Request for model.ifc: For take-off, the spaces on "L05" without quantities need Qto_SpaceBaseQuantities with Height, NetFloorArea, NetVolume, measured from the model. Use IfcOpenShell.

First a look at what the model holds.

```python
import ifcopenshell
import ifcopenshell.util.element
import ifcopenshell.util.unit

model = ifcopenshell.open("model.ifc")
print(model.schema)
for unit_type in ("LENGTHUNIT", "AREAUNIT", "VOLUMEUNIT"):
    print(unit_type, ifcopenshell.util.unit.calculate_unit_scale(model, unit_type))
storey = next(s for s in model.by_type("IfcBuildingStorey") if s.Name == "L05")
spaces = [e for e in ifcopenshell.util.element.get_decomposition(storey) if e.is_a("IfcSpace")]
for e in sorted(spaces, key=lambda e: e.id()):
    print(e.id(), e.is_a(), e.Name, list(ifcopenshell.util.element.get_psets(e, qtos_only=True)), sep=" | ")
```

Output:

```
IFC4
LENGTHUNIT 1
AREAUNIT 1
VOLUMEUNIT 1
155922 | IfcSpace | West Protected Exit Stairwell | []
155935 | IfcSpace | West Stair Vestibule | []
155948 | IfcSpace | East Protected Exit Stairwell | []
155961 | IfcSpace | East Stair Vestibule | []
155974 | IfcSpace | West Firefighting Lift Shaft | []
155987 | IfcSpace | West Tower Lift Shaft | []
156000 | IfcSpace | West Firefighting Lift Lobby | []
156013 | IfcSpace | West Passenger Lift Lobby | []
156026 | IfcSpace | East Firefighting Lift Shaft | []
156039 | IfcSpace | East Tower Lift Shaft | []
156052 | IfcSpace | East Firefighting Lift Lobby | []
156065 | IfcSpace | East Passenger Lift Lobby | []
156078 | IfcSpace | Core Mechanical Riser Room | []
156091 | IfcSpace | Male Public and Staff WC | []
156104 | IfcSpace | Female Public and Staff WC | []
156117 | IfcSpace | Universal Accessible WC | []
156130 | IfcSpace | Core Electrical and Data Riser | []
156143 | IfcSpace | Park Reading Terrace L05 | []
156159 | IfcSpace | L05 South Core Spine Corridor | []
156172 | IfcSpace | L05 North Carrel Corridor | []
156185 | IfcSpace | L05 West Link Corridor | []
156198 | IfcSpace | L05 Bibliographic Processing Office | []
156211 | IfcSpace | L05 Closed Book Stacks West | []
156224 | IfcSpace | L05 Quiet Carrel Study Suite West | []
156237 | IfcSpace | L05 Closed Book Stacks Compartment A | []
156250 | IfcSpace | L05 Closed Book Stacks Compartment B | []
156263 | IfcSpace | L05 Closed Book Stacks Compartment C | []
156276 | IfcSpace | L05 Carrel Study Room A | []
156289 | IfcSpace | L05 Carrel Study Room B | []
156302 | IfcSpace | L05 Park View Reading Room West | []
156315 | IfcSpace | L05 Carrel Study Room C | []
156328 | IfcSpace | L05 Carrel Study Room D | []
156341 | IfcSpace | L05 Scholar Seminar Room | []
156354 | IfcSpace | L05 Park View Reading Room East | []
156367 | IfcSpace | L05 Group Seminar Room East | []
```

```python
import ifcopenshell
import ifcopenshell.api.pset
import ifcopenshell.geom
import ifcopenshell.util.element
import ifcopenshell.util.shape
import ifcopenshell.util.unit

model = ifcopenshell.open("model.ifc")
unit_scale = ifcopenshell.util.unit.calculate_unit_scale(model)
area_scale = ifcopenshell.util.unit.calculate_unit_scale(model, "AREAUNIT")
volume_scale = ifcopenshell.util.unit.calculate_unit_scale(model, "VOLUMEUNIT")
settings = ifcopenshell.geom.settings()

storey = next(s for s in model.by_type("IfcBuildingStorey") if s.Name == "L05")
spaces = [e for e in ifcopenshell.util.element.get_decomposition(storey) if e.is_a("IfcSpace")]

for e in sorted(spaces, key=lambda e: e.id()):
    if ifcopenshell.util.element.get_psets(e, qtos_only=True, should_inherit=False):
        continue
    # Geometry comes back in metres, in the element's own axes.
    shape = ifcopenshell.geom.create_shape(settings, e)
    values = {
        "Height": ifcopenshell.util.shape.get_z(shape.geometry) / unit_scale,
        "NetFloorArea": ifcopenshell.util.shape.get_footprint_area(shape.geometry) / area_scale,
        "NetVolume": ifcopenshell.util.shape.get_volume(shape.geometry) / volume_scale,
    }
    qto = ifcopenshell.api.pset.add_qto(model, product=e, name="Qto_SpaceBaseQuantities")
    ifcopenshell.api.pset.edit_qto(model, qto=qto, properties=values)
    print(e.id(), {k: round(v, 3) for k, v in values.items()})

model.write("model_updated.ifc")
```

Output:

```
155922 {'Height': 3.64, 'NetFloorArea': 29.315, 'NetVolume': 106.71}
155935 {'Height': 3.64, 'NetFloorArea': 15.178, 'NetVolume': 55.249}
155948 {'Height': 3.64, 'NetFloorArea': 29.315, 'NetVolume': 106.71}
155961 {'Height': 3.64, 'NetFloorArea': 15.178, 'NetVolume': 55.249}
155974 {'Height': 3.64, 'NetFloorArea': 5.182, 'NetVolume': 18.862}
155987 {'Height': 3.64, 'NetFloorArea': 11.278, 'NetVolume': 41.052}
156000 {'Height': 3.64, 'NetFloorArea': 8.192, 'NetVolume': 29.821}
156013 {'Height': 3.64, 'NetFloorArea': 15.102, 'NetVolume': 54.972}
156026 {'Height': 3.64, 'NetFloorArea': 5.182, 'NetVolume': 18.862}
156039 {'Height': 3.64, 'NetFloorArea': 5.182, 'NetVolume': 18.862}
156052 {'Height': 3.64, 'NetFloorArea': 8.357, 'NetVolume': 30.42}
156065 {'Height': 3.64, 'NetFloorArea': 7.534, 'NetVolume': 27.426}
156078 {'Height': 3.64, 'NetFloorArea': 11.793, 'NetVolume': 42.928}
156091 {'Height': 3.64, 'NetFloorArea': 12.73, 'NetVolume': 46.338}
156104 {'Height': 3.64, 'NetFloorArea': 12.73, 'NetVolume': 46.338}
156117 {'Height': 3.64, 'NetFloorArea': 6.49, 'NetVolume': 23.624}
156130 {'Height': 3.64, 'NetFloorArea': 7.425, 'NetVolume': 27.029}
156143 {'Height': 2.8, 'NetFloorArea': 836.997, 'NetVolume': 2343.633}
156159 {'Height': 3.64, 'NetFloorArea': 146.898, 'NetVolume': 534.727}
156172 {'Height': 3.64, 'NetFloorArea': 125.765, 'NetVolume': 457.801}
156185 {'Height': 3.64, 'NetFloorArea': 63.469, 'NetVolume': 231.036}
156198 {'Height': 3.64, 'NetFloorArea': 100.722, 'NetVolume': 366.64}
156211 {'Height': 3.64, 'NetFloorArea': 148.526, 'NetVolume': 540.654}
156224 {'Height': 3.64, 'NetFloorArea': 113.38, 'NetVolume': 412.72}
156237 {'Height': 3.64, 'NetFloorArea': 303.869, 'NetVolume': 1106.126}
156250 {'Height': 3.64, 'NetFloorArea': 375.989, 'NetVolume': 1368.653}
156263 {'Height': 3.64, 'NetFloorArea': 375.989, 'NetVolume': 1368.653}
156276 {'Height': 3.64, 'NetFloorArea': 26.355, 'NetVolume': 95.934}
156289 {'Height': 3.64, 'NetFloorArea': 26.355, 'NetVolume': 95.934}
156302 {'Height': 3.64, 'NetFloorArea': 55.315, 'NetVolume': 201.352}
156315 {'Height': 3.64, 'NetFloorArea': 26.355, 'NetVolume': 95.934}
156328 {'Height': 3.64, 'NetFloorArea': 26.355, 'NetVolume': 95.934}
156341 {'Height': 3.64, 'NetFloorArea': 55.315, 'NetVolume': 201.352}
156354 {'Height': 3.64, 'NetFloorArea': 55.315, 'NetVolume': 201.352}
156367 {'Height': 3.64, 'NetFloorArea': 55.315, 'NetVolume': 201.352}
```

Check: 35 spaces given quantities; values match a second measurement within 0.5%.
